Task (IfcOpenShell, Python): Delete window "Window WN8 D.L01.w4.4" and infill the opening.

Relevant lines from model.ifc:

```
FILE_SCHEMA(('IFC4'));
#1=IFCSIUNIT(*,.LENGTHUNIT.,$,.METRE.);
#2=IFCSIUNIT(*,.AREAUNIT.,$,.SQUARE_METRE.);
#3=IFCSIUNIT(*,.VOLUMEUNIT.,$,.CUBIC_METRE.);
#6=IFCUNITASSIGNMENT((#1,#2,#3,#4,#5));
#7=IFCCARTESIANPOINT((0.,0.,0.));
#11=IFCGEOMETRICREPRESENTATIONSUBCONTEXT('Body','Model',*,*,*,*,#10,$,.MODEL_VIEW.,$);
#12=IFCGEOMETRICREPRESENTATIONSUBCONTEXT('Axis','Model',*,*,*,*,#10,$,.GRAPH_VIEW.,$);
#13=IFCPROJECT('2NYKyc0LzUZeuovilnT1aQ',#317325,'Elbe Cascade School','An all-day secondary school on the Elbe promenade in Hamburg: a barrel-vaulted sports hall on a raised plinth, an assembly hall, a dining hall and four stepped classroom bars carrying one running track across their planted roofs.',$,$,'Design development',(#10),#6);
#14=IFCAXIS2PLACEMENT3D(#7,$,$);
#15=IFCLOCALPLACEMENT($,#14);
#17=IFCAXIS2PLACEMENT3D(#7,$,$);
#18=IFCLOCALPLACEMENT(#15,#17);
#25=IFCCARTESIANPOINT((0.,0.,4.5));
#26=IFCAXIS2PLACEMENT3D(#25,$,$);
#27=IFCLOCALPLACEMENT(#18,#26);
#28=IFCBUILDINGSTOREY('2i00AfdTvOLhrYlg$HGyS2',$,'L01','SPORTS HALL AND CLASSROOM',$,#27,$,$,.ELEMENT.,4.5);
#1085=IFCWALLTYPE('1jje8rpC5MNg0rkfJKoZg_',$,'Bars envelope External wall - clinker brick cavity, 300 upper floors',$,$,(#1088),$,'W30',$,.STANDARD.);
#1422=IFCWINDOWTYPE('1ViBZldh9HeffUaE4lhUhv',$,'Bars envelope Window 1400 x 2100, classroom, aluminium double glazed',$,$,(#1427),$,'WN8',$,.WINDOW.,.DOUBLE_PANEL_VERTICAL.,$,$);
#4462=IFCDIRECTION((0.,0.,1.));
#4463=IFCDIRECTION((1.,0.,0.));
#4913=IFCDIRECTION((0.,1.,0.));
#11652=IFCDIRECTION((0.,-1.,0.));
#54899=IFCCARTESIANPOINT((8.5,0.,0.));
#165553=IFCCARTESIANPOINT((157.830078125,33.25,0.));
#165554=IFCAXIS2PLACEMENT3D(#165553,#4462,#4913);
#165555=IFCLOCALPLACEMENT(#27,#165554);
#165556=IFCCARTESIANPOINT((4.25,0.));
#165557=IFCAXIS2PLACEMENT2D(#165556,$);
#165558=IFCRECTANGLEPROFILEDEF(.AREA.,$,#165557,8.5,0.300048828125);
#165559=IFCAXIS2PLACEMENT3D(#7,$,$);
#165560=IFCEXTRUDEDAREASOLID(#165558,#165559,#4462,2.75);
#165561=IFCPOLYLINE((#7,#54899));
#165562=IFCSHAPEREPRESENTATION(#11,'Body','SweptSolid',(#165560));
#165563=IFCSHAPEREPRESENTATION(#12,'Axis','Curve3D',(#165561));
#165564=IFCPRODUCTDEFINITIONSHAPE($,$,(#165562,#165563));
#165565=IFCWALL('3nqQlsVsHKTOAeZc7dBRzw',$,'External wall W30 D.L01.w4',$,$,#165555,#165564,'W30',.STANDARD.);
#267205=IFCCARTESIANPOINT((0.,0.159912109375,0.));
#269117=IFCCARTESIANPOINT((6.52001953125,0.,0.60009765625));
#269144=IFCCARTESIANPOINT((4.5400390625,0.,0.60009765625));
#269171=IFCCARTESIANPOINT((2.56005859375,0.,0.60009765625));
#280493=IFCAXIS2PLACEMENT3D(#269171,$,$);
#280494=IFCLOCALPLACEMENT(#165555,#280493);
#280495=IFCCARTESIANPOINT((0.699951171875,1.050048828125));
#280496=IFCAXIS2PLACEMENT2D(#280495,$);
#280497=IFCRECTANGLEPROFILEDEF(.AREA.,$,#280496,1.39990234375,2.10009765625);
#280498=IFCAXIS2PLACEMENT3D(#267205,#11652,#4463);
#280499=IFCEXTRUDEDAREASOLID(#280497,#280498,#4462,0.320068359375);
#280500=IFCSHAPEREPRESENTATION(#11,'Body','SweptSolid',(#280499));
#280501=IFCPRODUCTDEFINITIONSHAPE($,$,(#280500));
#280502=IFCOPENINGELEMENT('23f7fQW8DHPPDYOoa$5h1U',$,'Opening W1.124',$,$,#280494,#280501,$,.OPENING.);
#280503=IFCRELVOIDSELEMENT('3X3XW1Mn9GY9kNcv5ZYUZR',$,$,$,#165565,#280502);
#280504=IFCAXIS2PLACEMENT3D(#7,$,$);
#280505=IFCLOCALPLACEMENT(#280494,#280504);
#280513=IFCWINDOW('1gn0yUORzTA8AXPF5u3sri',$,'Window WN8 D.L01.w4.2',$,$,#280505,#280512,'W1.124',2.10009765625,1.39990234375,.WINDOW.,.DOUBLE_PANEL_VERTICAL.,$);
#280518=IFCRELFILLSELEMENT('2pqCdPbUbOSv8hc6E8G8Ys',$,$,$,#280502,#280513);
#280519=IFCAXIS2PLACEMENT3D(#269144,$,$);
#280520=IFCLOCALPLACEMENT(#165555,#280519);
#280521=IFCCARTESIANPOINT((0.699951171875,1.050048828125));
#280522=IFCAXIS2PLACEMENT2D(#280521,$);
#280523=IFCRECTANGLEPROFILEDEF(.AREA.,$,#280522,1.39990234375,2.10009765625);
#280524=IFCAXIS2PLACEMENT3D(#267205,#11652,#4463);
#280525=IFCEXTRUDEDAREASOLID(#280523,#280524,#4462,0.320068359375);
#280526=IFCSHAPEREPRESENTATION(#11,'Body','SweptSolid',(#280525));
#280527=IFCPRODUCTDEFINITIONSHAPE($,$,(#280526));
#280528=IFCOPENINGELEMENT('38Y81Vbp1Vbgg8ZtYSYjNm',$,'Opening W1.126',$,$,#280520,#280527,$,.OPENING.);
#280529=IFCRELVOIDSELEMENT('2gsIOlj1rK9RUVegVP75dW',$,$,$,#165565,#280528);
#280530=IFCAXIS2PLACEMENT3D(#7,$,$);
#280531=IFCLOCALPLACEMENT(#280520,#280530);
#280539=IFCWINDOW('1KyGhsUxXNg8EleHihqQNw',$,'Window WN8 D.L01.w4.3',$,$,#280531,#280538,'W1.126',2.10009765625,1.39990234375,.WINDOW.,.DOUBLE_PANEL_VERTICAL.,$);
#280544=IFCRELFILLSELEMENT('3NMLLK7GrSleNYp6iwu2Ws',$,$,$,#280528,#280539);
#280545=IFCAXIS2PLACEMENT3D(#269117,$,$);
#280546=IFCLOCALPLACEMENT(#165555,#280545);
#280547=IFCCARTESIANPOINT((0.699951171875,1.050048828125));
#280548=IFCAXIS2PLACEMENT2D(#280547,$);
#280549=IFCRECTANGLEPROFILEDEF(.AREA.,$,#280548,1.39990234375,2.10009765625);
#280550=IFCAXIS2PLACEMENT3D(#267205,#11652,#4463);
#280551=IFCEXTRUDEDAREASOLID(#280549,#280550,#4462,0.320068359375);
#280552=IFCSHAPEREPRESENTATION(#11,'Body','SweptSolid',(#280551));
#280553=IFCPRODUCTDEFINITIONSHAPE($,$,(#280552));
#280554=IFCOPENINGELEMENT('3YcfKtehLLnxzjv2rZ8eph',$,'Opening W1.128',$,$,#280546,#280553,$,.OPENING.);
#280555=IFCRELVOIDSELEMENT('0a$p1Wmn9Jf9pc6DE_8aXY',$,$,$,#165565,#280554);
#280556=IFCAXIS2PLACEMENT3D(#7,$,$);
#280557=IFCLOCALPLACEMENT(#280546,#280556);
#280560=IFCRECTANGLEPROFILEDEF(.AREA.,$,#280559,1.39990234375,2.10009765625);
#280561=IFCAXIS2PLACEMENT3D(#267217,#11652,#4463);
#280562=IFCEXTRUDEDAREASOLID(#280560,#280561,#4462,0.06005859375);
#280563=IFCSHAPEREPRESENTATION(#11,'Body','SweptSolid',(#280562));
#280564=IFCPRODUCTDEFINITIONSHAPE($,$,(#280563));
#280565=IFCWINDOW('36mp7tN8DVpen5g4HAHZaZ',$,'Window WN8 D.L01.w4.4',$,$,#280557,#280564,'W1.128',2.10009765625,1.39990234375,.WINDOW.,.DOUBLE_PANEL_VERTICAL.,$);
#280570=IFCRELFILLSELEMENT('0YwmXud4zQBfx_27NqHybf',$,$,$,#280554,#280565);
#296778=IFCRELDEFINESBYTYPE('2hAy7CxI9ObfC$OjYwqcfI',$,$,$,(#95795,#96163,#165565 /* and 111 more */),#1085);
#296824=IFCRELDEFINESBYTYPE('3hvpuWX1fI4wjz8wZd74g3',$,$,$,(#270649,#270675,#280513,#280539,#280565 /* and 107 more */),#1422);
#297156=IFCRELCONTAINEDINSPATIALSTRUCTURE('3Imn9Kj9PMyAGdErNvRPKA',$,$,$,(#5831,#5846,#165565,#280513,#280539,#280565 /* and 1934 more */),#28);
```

```python
import ifcopenshell
import ifcopenshell.api.feature
import ifcopenshell.api.root
import ifcopenshell.geom
import ifcopenshell.util.shape

model = ifcopenshell.open("model.ifc")
settings = ifcopenshell.geom.settings()


def volume(element):
    """Net volume in cubic metres, openings subtracted."""
    shape = ifcopenshell.geom.create_shape(settings, element)
    return ifcopenshell.util.shape.get_volume(shape.geometry)


window = model.by_guid("36mp7tN8DVpen5g4HAHZaZ")
opening = window.FillsVoids[0].RelatingOpeningElement
wall = opening.VoidsElements[0].RelatingBuildingElement
before = volume(wall)

ifcopenshell.api.root.remove_product(model, product=window)
ifcopenshell.api.feature.remove_feature(model, feature=opening)

after = volume(wall)

print(f"wall volume {before:.3f} -> {after:.3f} m3")

model.write("model_edited.ifc")
```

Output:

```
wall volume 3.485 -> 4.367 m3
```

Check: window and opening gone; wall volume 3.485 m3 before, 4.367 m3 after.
